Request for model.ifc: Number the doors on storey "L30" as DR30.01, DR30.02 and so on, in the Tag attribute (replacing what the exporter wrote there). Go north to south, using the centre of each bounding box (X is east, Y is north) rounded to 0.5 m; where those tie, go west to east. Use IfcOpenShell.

First a look at what the model holds.

```python
import ifcopenshell
import ifcopenshell.util.element
import ifcopenshell.util.placement

model = ifcopenshell.open("model.ifc")
print(model.schema)
storey = next(s for s in model.by_type("IfcBuildingStorey") if s.Name == "L30")
doors = [e for e in ifcopenshell.util.element.get_decomposition(storey) if e.is_a("IfcDoor")]
for e in sorted(doors, key=lambda e: e.id()):
    origin = ifcopenshell.util.placement.get_local_placement(e.ObjectPlacement)[:3, 3]
    print(e.id(), e.Tag, e.Name, origin.round(2) + 0.0, sep=" | ")
```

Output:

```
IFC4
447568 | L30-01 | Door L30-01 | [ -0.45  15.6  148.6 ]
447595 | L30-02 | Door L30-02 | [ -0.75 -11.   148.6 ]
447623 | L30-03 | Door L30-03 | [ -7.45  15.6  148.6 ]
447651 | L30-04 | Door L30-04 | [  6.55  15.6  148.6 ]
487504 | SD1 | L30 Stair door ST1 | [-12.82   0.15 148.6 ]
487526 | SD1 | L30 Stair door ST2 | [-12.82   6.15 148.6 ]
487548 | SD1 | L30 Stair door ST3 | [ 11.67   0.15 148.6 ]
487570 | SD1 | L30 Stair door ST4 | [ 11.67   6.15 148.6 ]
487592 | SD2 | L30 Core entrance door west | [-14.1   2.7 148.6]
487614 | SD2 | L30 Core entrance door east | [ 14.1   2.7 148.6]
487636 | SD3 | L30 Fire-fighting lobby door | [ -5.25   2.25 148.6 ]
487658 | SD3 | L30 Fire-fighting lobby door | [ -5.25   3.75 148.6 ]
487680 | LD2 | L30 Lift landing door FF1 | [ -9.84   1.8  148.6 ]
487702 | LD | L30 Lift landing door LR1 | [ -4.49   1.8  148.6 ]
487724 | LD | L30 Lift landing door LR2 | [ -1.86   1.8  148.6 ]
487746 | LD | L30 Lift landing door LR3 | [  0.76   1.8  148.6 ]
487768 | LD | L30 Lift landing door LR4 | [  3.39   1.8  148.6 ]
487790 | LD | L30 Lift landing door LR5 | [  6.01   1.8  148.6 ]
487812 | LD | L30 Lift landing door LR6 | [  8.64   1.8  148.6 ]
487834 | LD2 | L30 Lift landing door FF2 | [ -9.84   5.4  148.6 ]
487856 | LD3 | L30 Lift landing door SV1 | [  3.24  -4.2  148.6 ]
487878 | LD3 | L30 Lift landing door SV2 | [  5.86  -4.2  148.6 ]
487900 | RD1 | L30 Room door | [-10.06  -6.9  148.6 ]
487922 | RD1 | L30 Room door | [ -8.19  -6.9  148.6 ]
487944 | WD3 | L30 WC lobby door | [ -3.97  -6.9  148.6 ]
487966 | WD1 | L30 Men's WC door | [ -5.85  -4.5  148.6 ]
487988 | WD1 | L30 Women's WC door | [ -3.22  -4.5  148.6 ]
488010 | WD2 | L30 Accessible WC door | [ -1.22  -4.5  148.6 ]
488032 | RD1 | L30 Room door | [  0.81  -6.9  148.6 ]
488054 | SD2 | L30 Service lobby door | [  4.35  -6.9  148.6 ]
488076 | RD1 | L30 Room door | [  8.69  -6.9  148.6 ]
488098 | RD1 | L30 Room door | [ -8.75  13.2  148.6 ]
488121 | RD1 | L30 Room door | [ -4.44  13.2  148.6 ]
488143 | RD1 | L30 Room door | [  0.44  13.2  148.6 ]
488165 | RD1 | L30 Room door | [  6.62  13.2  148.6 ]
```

```python
import ifcopenshell
import ifcopenshell.geom
import ifcopenshell.util.element
import ifcopenshell.util.shape

model = ifcopenshell.open("model.ifc")
settings = ifcopenshell.geom.settings()
settings.set("use-world-coords", True)


def centre(element):
    shape = ifcopenshell.geom.create_shape(settings, element)
    return ifcopenshell.util.shape.get_bbox_centroid(shape.geometry)


storey = next(s for s in model.by_type("IfcBuildingStorey") if s.Name == "L30")
doors = [e for e in ifcopenshell.util.element.get_decomposition(storey) if e.is_a("IfcDoor")]

# Insertion points can sit at a corner or the storey origin, so sort by the geometry (in metres).
centres = {e: centre(e) for e in doors}
doors.sort(key=lambda e: (-round(centres[e][1] / 0.5), centres[e][0]))

for i, e in enumerate(doors, start=1):
    number = f"DR30.{i:02d}"
    e.Tag = number
    print(e.id(), number)

model.write("model_rev.ifc")
```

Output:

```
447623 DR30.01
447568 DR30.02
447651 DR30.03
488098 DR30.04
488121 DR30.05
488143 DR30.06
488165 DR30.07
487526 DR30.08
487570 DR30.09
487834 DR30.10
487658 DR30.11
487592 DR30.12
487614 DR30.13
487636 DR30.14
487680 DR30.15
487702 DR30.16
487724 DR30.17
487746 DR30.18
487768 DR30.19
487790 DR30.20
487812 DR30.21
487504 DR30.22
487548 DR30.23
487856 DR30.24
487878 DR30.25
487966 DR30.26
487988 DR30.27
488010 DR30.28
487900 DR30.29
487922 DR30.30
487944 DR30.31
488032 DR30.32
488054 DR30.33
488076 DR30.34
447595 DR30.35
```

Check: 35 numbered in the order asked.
